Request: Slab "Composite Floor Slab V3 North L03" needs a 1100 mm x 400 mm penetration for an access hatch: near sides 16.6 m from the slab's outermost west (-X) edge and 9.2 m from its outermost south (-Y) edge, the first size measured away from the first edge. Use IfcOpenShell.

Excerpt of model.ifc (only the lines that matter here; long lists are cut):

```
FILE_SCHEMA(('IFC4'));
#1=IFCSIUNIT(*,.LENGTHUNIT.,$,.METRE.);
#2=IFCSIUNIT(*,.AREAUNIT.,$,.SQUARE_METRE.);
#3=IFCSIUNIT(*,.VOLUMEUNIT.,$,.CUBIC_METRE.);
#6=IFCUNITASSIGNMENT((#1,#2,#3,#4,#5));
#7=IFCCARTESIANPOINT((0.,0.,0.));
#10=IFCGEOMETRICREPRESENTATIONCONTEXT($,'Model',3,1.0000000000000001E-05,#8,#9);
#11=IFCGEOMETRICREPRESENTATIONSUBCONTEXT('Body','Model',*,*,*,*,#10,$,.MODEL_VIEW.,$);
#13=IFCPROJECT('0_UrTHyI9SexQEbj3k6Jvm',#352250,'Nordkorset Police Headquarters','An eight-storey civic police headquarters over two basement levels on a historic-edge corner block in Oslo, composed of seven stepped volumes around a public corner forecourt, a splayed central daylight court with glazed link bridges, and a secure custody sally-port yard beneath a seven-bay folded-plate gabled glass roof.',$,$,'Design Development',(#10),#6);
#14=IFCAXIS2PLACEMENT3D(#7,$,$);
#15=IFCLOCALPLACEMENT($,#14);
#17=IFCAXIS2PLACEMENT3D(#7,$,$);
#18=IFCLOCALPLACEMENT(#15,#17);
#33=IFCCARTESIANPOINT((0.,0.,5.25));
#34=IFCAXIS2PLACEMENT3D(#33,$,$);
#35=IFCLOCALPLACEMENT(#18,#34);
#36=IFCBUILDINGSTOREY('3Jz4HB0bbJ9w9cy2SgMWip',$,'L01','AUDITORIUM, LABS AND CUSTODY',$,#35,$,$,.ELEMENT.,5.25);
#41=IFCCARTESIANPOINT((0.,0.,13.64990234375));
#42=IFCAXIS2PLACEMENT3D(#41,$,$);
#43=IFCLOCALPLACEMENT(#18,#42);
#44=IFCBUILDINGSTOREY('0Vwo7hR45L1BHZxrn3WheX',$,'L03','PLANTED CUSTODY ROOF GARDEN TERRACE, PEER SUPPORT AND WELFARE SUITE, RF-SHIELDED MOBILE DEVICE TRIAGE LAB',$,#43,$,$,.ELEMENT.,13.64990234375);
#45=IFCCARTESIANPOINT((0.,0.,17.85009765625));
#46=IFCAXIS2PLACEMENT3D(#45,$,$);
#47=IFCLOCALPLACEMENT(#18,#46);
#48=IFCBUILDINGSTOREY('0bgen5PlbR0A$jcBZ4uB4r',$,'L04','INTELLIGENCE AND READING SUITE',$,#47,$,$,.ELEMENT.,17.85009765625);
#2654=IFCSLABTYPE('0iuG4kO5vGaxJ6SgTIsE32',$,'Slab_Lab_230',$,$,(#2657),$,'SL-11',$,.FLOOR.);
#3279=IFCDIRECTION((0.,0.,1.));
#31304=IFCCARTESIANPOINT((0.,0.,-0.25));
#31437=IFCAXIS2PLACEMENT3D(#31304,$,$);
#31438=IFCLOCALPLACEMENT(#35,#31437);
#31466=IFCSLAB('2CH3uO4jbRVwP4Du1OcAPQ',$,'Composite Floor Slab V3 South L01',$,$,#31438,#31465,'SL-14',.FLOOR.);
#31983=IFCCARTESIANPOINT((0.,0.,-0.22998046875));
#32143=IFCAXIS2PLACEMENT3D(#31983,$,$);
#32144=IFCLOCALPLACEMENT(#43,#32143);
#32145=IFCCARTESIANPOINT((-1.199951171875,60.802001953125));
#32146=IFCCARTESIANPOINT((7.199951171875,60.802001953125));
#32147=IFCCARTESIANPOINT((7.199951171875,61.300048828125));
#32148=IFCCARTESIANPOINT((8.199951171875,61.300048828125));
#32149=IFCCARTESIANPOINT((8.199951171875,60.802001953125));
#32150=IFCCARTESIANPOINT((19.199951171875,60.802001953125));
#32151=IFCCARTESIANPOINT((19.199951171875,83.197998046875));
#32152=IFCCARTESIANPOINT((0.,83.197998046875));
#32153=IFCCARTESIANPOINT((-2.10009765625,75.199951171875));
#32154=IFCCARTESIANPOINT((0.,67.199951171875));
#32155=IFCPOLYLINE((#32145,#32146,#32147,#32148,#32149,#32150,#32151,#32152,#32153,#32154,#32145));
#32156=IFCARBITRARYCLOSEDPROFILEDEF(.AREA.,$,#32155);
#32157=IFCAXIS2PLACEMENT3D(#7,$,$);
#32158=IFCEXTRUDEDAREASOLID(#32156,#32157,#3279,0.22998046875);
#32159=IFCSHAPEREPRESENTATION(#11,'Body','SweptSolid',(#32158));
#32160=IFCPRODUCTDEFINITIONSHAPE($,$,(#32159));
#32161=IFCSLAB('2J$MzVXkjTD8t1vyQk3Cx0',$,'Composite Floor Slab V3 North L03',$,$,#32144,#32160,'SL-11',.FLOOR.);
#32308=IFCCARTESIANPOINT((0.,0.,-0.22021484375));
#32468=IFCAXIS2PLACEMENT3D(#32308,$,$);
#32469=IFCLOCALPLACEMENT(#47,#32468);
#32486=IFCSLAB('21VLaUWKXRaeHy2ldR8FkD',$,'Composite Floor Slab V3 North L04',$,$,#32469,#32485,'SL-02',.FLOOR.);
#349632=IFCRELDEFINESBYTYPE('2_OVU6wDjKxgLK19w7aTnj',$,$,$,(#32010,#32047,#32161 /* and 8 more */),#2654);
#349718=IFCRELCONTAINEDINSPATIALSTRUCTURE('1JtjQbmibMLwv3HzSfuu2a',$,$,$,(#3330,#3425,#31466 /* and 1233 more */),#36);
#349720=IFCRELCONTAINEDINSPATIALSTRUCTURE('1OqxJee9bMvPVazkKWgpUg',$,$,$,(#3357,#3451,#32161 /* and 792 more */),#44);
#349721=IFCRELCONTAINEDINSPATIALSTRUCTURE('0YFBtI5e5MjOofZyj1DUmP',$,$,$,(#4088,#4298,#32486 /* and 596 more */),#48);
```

```python
import numpy as np
import ifcopenshell
import ifcopenshell.api.feature
import ifcopenshell.api.geometry
import ifcopenshell.api.root
import ifcopenshell.geom
import ifcopenshell.util.placement
import ifcopenshell.util.representation
import ifcopenshell.util.shape
import ifcopenshell.util.unit

model = ifcopenshell.open("model.ifc")
unit_scale = ifcopenshell.util.unit.calculate_unit_scale(model)
settings = ifcopenshell.geom.settings()


def volume(element):
    """Net volume in cubic metres, openings subtracted."""
    shape = ifcopenshell.geom.create_shape(settings, element)
    return ifcopenshell.util.shape.get_volume(shape.geometry)


slab = model.by_guid("2J$MzVXkjTD8t1vyQk3Cx0")
before = volume(slab)

# Extent in the slab's own axes, in metres. The edges named are its -X and -Y sides.
slab_shape = ifcopenshell.geom.create_shape(settings, slab)
vertices = ifcopenshell.util.shape.get_vertices(slab_shape.geometry)
x_min, y_min, bottom = vertices.min(axis=0)
top = vertices[:, 2].max()

opening = ifcopenshell.api.root.create_entity(model, ifc_class="IfcOpeningElement", name="Access hatch opening", predefined_type="OPENING")
context = ifcopenshell.util.representation.get_context(model, "Model", "Body", "MODEL_VIEW")
width, depth = 1.1, 0.4
outline = [(0.0, 0.0), (width, 0.0), (width, depth), (0.0, depth), (0.0, 0.0)]
# Overshoot both faces by 50 mm so the cut is clean.
shape = ifcopenshell.api.geometry.add_slab_representation(
    model, context=context, depth=top - bottom + 0.1, polyline=outline
)
ifcopenshell.api.geometry.assign_representation(model, product=opening, representation=shape)

matrix = ifcopenshell.util.placement.get_local_placement(slab.ObjectPlacement)
matrix[:, 3] = matrix @ np.append(np.array([x_min + 16.6, y_min + 9.2, bottom - 0.05]) / unit_scale, 1.0)
ifcopenshell.api.geometry.edit_object_placement(model, product=opening, matrix=matrix, is_si=False)
ifcopenshell.api.feature.add_feature(model, feature=opening, element=slab)

after = volume(slab)

print(f"slab volume {before:.3f} -> {after:.3f} m3")

model.write("model_v2.ifc")
```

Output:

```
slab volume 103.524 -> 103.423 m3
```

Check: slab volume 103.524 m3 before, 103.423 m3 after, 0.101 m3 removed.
